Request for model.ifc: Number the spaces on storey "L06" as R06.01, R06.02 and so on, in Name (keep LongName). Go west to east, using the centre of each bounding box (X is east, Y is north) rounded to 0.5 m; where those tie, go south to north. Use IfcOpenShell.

First a look at what the model holds.

```python
import ifcopenshell
import ifcopenshell.util.element
import ifcopenshell.util.placement

model = ifcopenshell.open("model.ifc")
print(model.schema)
storey = next(s for s in model.by_type("IfcBuildingStorey") if s.Name == "L06")
spaces = [e for e in ifcopenshell.util.element.get_decomposition(storey) if e.is_a("IfcSpace")]
for e in sorted(spaces, key=lambda e: e.id()):
    origin = ifcopenshell.util.placement.get_local_placement(e.ObjectPlacement)[:3, 3]
    print(e.id(), e.Name, e.LongName, origin.round(2) + 0.0, sep=" | ")
```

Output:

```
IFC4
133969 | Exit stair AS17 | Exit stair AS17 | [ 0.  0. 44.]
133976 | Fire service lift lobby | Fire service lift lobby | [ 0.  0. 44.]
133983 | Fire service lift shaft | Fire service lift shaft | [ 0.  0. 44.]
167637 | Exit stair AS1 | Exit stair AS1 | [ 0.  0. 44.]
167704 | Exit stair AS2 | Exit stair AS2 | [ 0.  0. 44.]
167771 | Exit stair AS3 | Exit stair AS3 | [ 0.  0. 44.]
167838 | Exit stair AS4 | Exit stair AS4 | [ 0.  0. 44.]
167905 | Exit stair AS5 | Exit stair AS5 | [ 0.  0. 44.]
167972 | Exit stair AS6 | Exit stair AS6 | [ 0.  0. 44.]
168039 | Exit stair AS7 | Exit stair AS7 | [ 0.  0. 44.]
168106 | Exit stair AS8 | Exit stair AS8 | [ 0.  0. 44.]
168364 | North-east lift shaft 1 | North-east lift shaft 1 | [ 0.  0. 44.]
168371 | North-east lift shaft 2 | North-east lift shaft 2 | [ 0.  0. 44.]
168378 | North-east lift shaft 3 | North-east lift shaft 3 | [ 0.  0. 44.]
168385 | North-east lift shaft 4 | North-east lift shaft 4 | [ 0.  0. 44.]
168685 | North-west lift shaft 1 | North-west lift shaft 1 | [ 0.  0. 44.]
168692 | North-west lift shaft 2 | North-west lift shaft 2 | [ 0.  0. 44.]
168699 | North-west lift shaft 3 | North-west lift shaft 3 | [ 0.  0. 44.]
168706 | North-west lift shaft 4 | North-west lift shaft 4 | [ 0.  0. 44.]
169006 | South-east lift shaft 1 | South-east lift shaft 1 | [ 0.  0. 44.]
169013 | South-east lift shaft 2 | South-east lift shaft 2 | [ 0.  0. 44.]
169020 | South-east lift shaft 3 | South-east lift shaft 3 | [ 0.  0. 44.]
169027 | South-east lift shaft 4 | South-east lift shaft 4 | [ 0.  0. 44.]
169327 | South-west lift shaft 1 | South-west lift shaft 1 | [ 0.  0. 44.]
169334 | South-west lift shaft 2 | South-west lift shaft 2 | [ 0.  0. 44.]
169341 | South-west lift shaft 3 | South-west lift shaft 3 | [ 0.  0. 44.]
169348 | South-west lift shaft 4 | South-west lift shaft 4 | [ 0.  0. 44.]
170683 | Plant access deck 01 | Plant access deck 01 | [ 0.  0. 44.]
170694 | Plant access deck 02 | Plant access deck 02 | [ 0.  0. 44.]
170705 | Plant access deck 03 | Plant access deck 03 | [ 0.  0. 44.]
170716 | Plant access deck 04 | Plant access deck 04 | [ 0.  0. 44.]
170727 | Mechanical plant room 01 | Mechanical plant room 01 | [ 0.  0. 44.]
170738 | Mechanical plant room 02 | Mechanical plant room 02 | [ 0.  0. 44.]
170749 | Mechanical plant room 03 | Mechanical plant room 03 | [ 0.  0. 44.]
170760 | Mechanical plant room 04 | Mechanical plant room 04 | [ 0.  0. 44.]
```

```python
import ifcopenshell
import ifcopenshell.geom
import ifcopenshell.util.element
import ifcopenshell.util.shape

model = ifcopenshell.open("model.ifc")
settings = ifcopenshell.geom.settings()
settings.set("use-world-coords", True)


def centre(element):
    shape = ifcopenshell.geom.create_shape(settings, element)
    return ifcopenshell.util.shape.get_bbox_centroid(shape.geometry)


storey = next(s for s in model.by_type("IfcBuildingStorey") if s.Name == "L06")
spaces = [e for e in ifcopenshell.util.element.get_decomposition(storey) if e.is_a("IfcSpace")]

# Insertion points can sit at a corner or the storey origin, so sort by the geometry (in metres).
centres = {e: centre(e) for e in spaces}
spaces.sort(key=lambda e: (round(centres[e][0] / 0.5), centres[e][1]))

for i, e in enumerate(spaces, start=1):
    number = f"R06.{i:02d}"
    e.Name = number
    print(e.id(), number)

model.write("model_v2.ifc")
```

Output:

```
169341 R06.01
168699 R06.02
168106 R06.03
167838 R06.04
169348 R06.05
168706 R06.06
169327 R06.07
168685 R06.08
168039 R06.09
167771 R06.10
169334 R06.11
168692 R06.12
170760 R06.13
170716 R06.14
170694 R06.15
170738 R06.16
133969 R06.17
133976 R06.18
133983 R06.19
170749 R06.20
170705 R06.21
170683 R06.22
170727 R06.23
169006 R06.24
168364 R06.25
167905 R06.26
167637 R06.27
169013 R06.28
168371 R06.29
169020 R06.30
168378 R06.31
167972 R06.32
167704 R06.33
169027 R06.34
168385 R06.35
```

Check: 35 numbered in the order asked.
